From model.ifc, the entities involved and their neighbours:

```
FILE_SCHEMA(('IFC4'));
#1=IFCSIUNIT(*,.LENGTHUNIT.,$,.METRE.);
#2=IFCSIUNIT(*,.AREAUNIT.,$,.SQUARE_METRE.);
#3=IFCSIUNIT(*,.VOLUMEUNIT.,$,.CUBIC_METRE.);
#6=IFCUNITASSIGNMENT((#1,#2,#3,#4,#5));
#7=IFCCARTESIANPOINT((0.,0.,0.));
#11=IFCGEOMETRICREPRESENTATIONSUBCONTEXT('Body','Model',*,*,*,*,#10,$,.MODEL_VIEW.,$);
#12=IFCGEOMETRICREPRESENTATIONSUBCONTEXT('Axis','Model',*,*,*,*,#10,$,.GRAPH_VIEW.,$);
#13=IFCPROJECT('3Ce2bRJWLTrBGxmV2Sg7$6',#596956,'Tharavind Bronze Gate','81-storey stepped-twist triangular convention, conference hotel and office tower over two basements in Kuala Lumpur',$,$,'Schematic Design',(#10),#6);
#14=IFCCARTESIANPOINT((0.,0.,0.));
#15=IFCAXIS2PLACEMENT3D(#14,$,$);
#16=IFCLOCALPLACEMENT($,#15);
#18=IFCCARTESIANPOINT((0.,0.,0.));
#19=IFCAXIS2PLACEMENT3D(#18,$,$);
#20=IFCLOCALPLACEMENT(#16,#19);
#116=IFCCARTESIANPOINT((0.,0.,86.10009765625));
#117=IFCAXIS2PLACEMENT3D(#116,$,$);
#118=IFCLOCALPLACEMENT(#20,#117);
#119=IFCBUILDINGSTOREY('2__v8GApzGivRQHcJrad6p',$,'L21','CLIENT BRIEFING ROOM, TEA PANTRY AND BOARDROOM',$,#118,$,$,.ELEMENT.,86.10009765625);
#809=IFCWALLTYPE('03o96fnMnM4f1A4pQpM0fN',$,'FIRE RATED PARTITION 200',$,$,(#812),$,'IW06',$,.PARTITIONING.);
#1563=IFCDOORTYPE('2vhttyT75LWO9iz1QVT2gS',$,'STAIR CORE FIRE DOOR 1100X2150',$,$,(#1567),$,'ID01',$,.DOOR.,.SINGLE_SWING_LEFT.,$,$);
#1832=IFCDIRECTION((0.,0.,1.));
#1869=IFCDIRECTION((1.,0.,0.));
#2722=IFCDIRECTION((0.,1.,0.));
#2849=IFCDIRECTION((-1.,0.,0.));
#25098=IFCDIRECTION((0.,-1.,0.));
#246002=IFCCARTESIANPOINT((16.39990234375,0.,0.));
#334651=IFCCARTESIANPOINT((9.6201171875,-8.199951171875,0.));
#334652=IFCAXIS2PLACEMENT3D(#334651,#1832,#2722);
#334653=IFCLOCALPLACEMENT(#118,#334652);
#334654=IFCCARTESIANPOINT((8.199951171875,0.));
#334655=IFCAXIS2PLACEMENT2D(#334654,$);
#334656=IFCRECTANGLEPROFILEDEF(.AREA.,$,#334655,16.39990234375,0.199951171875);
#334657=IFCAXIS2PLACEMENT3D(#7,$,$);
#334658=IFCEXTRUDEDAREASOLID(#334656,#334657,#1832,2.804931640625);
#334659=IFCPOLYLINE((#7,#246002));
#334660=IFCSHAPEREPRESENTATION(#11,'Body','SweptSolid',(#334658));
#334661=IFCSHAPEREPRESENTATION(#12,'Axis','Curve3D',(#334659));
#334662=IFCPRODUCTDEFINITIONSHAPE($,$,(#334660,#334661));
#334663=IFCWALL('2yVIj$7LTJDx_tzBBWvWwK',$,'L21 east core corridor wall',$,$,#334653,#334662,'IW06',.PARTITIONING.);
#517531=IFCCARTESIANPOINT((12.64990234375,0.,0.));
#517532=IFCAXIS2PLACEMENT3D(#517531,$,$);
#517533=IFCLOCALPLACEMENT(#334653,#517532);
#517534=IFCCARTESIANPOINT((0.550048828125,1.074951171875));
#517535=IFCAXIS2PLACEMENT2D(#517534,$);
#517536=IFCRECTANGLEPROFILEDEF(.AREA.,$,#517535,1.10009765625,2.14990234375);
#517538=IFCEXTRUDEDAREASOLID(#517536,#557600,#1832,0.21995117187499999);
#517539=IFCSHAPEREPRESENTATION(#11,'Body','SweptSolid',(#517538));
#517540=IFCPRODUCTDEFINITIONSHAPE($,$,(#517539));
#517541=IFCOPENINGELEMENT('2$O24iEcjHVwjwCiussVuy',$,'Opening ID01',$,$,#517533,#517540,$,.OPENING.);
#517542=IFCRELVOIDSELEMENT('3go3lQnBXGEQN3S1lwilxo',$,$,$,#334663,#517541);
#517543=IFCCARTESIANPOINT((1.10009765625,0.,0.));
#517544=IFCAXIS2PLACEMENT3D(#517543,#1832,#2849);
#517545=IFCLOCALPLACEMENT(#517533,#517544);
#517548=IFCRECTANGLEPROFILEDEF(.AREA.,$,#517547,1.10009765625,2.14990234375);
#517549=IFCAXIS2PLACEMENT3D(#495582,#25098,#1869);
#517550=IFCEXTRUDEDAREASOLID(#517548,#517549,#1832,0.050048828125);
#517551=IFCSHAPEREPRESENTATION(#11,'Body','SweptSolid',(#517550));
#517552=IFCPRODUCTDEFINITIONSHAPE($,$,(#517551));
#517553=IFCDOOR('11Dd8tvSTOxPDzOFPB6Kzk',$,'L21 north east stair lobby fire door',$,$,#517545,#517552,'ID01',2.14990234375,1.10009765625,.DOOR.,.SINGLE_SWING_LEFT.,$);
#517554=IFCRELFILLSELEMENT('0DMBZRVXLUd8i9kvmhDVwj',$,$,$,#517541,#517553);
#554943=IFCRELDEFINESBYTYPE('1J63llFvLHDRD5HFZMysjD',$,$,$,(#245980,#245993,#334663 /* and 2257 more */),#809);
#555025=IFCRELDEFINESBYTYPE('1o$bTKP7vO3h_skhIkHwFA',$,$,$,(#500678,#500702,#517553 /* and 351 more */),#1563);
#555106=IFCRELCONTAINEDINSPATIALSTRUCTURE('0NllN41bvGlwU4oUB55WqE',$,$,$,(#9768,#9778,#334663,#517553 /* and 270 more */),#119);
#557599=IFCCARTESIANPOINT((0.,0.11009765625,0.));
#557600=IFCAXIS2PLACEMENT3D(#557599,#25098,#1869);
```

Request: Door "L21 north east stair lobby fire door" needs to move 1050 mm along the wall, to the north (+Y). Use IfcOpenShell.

```python
import ifcopenshell
import ifcopenshell.api.geometry
import ifcopenshell.util.placement
import ifcopenshell.util.unit

model = ifcopenshell.open("model.ifc")
unit_scale = ifcopenshell.util.unit.calculate_unit_scale(model)

door = model.by_guid("11Dd8tvSTOxPDzOFPB6Kzk")
opening = door.FillsVoids[0].RelatingOpeningElement
wall = opening.VoidsElements[0].RelatingBuildingElement

wall_matrix = ifcopenshell.util.placement.get_local_placement(wall.ObjectPlacement)
shift = wall_matrix[:3, 0] * 1.05 / unit_scale
before = ifcopenshell.util.placement.get_local_placement(door.ObjectPlacement)[:3, 3].copy()

# The door is placed relative to its opening, so it follows when the opening moves.
matrix = ifcopenshell.util.placement.get_local_placement(opening.ObjectPlacement)
matrix[:3, 3] += shift
ifcopenshell.api.geometry.edit_object_placement(
    model, product=opening, matrix=matrix, is_si=False, should_transform_children=True
)

after = ifcopenshell.util.placement.get_local_placement(door.ObjectPlacement)[:3, 3]
print("door moved by", (after - before).round(3) + 0.0)

model.write("model_rev.ifc")
```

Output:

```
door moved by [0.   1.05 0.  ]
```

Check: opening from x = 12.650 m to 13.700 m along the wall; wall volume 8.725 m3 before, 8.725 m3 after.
